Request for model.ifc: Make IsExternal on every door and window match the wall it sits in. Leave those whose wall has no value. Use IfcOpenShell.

First a look at what the model holds.

```python
import ifcopenshell
import ifcopenshell.util.element

model = ifcopenshell.open("model.ifc")
print(model.schema)
seen = {}
for e in model.by_type("IfcDoor") + model.by_type("IfcWindow"):
    if not e.FillsVoids:
        continue
    host = e.FillsVoids[0].RelatingOpeningElement.VoidsElements[0].RelatingBuildingElement
    own = ifcopenshell.util.element.get_pset(e, f"Pset_{e.is_a()[3:].removesuffix('StandardCase')}Common", "IsExternal")
    wall = ifcopenshell.util.element.get_pset(host, "Pset_WallCommon", "IsExternal")
    seen[e.is_a(), own, wall] = seen.get((e.is_a(), own, wall), 0) + 1
for (cls, own, wall), count in sorted(seen.items(), key=str):
    print(count, cls, "IsExternal:", own, "| host wall:", wall)
```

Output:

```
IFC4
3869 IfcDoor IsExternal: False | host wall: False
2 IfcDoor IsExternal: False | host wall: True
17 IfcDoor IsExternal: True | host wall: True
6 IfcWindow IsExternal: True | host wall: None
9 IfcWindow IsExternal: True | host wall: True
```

```python
import ifcopenshell
import ifcopenshell.api.pset
import ifcopenshell.util.element

model = ifcopenshell.open("model.ifc")

count = 0
for ifc_class, pset_name in (("IfcDoor", "Pset_DoorCommon"), ("IfcWindow", "Pset_WindowCommon")):
    for e in model.by_type(ifc_class):
        if not e.FillsVoids:
            continue
        host = e.FillsVoids[0].RelatingOpeningElement.VoidsElements[0].RelatingBuildingElement
        external = ifcopenshell.util.element.get_pset(host, "Pset_WallCommon", "IsExternal")
        if external is None or ifcopenshell.util.element.get_pset(e, pset_name, "IsExternal") == external:
            continue
        pset = ifcopenshell.api.pset.add_pset(model, product=e, name=pset_name)
        ifcopenshell.api.pset.edit_pset(model, pset=pset, properties={"IsExternal": external})
        count += 1

print(count, "updated")

model.write("model_rev.ifc")
```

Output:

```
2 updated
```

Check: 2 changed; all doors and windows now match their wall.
